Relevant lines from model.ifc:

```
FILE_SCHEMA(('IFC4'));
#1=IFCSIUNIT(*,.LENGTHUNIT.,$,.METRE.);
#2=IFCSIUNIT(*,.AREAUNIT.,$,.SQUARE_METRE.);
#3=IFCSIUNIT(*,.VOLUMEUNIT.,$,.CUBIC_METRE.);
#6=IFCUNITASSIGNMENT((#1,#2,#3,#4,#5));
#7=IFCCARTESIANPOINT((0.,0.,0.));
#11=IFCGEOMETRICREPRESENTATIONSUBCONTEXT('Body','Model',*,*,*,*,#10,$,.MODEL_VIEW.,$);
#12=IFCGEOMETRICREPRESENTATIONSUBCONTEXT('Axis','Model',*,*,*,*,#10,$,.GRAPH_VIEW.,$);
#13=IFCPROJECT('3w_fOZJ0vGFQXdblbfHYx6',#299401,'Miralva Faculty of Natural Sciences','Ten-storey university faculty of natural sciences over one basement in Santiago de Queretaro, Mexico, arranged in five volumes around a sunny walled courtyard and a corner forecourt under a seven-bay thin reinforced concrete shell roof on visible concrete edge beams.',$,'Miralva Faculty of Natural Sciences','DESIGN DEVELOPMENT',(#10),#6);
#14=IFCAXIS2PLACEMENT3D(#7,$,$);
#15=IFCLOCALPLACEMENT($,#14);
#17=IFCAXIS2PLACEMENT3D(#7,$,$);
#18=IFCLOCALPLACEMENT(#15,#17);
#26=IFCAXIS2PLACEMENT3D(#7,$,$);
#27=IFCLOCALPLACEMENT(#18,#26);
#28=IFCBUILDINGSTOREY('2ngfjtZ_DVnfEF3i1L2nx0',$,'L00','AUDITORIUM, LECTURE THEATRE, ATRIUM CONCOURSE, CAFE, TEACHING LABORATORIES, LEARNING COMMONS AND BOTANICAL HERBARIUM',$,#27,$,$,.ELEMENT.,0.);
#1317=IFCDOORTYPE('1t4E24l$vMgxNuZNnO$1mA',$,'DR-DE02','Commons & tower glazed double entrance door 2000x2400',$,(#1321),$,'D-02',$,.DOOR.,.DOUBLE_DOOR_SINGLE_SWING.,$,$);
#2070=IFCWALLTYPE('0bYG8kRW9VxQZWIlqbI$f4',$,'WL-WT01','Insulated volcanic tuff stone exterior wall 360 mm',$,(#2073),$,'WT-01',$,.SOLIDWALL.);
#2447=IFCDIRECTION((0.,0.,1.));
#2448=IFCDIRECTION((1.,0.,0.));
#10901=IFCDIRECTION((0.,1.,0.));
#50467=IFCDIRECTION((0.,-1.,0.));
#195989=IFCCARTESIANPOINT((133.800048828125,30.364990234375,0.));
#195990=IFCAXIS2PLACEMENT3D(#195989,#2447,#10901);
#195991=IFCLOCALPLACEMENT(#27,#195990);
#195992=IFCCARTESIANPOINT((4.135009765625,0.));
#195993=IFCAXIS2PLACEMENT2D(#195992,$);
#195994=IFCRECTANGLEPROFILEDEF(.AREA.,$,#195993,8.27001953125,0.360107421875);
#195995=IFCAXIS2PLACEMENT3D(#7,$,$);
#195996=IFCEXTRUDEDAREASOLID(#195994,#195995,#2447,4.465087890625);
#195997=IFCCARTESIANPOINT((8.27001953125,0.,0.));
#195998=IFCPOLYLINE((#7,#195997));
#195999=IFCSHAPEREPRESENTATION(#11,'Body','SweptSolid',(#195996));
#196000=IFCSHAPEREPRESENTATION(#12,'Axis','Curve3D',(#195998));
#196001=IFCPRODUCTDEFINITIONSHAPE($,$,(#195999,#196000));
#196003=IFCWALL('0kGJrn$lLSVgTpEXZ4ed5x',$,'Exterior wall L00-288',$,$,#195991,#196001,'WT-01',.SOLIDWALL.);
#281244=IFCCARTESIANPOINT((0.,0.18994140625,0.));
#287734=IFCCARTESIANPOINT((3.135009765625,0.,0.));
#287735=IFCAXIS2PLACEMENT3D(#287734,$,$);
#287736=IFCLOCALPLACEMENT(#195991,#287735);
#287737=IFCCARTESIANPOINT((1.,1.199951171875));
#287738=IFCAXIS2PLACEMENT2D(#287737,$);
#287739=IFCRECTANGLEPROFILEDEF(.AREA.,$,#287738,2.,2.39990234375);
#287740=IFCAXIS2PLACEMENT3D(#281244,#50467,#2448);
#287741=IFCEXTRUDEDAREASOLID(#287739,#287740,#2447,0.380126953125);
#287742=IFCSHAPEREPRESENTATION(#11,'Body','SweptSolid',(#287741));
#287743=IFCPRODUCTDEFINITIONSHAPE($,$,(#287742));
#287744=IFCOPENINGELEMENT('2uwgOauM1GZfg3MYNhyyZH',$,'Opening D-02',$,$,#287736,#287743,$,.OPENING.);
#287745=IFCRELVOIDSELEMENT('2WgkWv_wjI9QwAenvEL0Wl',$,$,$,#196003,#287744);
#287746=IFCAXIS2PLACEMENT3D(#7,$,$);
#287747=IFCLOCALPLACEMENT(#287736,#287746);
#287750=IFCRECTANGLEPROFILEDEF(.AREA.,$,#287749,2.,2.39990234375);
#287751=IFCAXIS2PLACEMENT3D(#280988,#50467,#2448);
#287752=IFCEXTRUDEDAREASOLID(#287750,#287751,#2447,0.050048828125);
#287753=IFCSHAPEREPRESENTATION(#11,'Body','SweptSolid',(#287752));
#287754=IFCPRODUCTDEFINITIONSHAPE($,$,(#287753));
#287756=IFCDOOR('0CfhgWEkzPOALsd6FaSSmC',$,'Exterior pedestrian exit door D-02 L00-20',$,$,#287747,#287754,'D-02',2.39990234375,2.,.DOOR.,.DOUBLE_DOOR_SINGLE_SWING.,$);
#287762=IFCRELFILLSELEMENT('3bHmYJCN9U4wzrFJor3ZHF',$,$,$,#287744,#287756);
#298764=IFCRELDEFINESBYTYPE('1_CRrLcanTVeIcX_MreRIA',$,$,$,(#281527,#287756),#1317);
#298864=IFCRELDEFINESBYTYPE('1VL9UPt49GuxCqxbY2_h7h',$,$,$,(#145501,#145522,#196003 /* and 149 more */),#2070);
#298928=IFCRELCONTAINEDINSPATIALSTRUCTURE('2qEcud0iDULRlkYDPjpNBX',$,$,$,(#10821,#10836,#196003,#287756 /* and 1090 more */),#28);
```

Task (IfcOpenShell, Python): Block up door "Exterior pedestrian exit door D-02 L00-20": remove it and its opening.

```python
import ifcopenshell
import ifcopenshell.api.feature
import ifcopenshell.api.root
import ifcopenshell.geom
import ifcopenshell.util.shape

model = ifcopenshell.open("model.ifc")
settings = ifcopenshell.geom.settings()


def volume(element):
    """Net volume in cubic metres, openings subtracted."""
    shape = ifcopenshell.geom.create_shape(settings, element)
    return ifcopenshell.util.shape.get_volume(shape.geometry)


door = model.by_id(287756)
opening = door.FillsVoids[0].RelatingOpeningElement
wall = opening.VoidsElements[0].RelatingBuildingElement
before = volume(wall)

ifcopenshell.api.root.remove_product(model, product=door)
ifcopenshell.api.feature.remove_feature(model, feature=opening)

after = volume(wall)

print(f"wall volume {before:.3f} -> {after:.3f} m3")

model.write("model_rev.ifc")
```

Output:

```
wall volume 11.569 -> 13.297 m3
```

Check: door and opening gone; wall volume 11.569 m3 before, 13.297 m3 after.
